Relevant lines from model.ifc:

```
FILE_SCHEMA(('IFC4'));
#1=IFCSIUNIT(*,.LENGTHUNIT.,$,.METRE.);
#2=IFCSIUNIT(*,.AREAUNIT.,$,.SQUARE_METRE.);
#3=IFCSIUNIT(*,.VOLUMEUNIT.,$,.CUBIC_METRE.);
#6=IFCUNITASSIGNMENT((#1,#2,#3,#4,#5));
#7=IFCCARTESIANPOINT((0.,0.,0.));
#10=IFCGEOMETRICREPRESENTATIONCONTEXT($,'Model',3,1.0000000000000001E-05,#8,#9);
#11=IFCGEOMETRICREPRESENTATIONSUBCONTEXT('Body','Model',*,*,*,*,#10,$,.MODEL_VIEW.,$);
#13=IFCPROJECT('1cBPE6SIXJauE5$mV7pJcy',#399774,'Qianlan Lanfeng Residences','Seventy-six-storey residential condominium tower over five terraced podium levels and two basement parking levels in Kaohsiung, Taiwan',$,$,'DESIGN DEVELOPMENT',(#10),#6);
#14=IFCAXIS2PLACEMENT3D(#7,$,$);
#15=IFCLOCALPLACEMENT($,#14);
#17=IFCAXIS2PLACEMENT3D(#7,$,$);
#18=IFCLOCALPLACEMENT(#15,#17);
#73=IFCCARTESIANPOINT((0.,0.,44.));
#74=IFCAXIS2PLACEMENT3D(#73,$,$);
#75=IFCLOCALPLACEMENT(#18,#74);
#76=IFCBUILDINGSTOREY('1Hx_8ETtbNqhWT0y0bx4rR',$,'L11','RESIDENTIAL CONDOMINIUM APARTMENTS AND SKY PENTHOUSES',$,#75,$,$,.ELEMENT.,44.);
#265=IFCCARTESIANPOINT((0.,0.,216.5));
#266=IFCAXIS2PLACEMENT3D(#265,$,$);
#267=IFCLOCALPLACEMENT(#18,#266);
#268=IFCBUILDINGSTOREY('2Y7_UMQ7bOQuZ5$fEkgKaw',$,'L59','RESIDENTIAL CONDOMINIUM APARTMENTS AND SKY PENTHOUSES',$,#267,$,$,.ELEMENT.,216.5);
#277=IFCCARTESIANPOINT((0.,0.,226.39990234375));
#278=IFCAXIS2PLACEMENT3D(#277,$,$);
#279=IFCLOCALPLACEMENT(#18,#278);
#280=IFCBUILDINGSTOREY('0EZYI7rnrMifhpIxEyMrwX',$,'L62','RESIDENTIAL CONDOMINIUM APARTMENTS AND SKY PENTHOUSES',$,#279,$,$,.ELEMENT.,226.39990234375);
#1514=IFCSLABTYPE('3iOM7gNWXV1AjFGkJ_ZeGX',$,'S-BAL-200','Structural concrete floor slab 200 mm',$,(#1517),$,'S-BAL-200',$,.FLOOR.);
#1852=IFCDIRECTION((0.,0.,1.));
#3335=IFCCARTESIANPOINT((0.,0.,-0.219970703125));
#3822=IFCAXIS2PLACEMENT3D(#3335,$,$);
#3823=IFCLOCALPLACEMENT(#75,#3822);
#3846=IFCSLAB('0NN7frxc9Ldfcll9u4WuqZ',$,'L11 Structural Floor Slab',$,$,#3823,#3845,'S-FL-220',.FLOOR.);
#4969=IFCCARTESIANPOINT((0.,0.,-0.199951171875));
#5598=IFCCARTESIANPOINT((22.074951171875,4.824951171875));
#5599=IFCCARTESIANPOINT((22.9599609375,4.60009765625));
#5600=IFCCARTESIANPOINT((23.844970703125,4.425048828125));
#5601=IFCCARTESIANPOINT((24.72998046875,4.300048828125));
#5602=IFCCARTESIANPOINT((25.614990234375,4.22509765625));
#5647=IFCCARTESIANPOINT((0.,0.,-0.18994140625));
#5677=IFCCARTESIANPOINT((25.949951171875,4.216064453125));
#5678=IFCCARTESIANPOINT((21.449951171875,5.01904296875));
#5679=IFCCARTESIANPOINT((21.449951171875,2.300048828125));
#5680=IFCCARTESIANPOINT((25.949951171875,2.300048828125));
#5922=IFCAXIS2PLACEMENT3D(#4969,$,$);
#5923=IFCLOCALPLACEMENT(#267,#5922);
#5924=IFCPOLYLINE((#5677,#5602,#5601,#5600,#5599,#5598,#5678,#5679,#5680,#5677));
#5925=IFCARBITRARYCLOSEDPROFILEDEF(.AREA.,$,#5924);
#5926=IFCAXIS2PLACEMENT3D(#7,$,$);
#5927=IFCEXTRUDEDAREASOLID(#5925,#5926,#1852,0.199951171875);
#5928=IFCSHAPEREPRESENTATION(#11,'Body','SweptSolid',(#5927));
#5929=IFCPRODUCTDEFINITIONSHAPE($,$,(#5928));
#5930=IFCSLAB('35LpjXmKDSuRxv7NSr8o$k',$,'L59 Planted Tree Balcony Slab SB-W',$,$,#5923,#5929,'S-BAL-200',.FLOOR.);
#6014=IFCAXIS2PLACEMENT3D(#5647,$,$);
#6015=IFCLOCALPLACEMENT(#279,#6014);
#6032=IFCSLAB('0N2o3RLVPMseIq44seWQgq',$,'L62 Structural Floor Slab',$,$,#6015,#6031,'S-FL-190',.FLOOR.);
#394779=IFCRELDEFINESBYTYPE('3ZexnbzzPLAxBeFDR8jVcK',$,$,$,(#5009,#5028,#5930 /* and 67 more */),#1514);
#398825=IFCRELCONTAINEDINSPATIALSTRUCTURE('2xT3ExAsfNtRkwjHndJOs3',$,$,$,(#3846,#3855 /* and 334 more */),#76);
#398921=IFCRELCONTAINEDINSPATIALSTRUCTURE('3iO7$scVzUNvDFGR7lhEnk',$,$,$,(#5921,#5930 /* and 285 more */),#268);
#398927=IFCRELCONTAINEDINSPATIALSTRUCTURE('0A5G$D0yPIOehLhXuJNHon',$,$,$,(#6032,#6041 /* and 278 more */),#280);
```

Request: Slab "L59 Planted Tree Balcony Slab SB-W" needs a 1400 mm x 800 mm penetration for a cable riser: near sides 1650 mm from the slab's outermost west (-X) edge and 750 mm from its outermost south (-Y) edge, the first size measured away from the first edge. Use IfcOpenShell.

```python
import numpy as np
import ifcopenshell
import ifcopenshell.api.feature
import ifcopenshell.api.geometry
import ifcopenshell.api.root
import ifcopenshell.geom
import ifcopenshell.util.placement
import ifcopenshell.util.representation
import ifcopenshell.util.shape
import ifcopenshell.util.unit

model = ifcopenshell.open("model.ifc")
unit_scale = ifcopenshell.util.unit.calculate_unit_scale(model)
settings = ifcopenshell.geom.settings()


def volume(element):
    """Net volume in cubic metres, openings subtracted."""
    shape = ifcopenshell.geom.create_shape(settings, element)
    return ifcopenshell.util.shape.get_volume(shape.geometry)


slab = model.by_guid("35LpjXmKDSuRxv7NSr8o$k")
before = volume(slab)

# Extent in the slab's own axes, in metres. The edges named are its -X and -Y sides.
slab_shape = ifcopenshell.geom.create_shape(settings, slab)
vertices = ifcopenshell.util.shape.get_vertices(slab_shape.geometry)
x_min, y_min, bottom = vertices.min(axis=0)
top = vertices[:, 2].max()

opening = ifcopenshell.api.root.create_entity(model, ifc_class="IfcOpeningElement", name="Cable riser opening", predefined_type="OPENING")
context = ifcopenshell.util.representation.get_context(model, "Model", "Body", "MODEL_VIEW")
width, depth = 1.4, 0.8
outline = [(0.0, 0.0), (width, 0.0), (width, depth), (0.0, depth), (0.0, 0.0)]
# Overshoot both faces by 50 mm so the cut is clean.
shape = ifcopenshell.api.geometry.add_slab_representation(
    model, context=context, depth=top - bottom + 0.1, polyline=outline
)
ifcopenshell.api.geometry.assign_representation(model, product=opening, representation=shape)

matrix = ifcopenshell.util.placement.get_local_placement(slab.ObjectPlacement)
matrix[:, 3] = matrix @ np.append(np.array([x_min + 1.65, y_min + 0.75, bottom - 0.05]) / unit_scale, 1.0)
ifcopenshell.api.geometry.edit_object_placement(model, product=opening, matrix=matrix, is_si=False)
ifcopenshell.api.feature.add_feature(model, feature=opening, element=slab)

after = volume(slab)

print(f"slab volume {before:.3f} -> {after:.3f} m3")

model.write("model_updated.ifc")
```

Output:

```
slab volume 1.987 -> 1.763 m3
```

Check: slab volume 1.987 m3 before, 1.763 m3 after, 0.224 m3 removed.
